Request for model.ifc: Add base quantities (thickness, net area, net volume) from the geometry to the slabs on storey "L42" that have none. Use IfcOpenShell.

First a look at what the model holds.

```python
import ifcopenshell
import ifcopenshell.util.element
import ifcopenshell.util.unit

model = ifcopenshell.open("model.ifc")
print(model.schema)
for unit_type in ("LENGTHUNIT", "AREAUNIT", "VOLUMEUNIT"):
    print(unit_type, ifcopenshell.util.unit.calculate_unit_scale(model, unit_type))
storey = next(s for s in model.by_type("IfcBuildingStorey") if s.Name == "L42")
slabs = [e for e in ifcopenshell.util.element.get_decomposition(storey) if e.is_a("IfcSlab")]
for e in sorted(slabs, key=lambda e: e.id()):
    print(e.id(), e.is_a(), e.Name, list(ifcopenshell.util.element.get_psets(e, qtos_only=True)), sep=" | ")
```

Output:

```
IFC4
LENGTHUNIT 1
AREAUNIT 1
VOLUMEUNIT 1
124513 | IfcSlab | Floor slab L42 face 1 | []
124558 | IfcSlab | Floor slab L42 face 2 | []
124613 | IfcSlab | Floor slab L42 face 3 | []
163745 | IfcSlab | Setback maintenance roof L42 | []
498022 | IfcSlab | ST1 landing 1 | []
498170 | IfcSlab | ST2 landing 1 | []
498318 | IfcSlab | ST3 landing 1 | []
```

```python
import ifcopenshell
import ifcopenshell.api.pset
import ifcopenshell.geom
import ifcopenshell.util.element
import ifcopenshell.util.shape
import ifcopenshell.util.unit

model = ifcopenshell.open("model.ifc")
unit_scale = ifcopenshell.util.unit.calculate_unit_scale(model)
area_scale = ifcopenshell.util.unit.calculate_unit_scale(model, "AREAUNIT")
volume_scale = ifcopenshell.util.unit.calculate_unit_scale(model, "VOLUMEUNIT")
settings = ifcopenshell.geom.settings()

storey = next(s for s in model.by_type("IfcBuildingStorey") if s.Name == "L42")
slabs = [e for e in ifcopenshell.util.element.get_decomposition(storey) if e.is_a("IfcSlab")]

for e in sorted(slabs, key=lambda e: e.id()):
    if ifcopenshell.util.element.get_psets(e, qtos_only=True, should_inherit=False):
        continue
    # Geometry comes back in metres, in the element's own axes.
    shape = ifcopenshell.geom.create_shape(settings, e)
    values = {
        "Width": ifcopenshell.util.shape.get_z(shape.geometry) / unit_scale,
        "NetArea": ifcopenshell.util.shape.get_footprint_area(shape.geometry) / area_scale,
        "NetVolume": ifcopenshell.util.shape.get_volume(shape.geometry) / volume_scale,
    }
    qto = ifcopenshell.api.pset.add_qto(model, product=e, name="Qto_SlabBaseQuantities")
    ifcopenshell.api.pset.edit_qto(model, qto=qto, properties=values)
    print(e.id(), {k: round(v, 3) for k, v in values.items()})

model.write("model-out.ifc")
```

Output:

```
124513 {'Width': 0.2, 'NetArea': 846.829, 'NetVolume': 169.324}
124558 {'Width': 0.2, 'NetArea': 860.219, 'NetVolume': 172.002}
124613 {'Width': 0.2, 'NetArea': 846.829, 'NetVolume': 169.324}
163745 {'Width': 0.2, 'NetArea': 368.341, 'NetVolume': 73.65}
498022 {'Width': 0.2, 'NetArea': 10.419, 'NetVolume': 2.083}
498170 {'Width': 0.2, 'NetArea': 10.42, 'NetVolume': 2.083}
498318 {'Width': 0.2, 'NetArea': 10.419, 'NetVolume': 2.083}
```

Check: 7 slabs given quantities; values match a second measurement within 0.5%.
